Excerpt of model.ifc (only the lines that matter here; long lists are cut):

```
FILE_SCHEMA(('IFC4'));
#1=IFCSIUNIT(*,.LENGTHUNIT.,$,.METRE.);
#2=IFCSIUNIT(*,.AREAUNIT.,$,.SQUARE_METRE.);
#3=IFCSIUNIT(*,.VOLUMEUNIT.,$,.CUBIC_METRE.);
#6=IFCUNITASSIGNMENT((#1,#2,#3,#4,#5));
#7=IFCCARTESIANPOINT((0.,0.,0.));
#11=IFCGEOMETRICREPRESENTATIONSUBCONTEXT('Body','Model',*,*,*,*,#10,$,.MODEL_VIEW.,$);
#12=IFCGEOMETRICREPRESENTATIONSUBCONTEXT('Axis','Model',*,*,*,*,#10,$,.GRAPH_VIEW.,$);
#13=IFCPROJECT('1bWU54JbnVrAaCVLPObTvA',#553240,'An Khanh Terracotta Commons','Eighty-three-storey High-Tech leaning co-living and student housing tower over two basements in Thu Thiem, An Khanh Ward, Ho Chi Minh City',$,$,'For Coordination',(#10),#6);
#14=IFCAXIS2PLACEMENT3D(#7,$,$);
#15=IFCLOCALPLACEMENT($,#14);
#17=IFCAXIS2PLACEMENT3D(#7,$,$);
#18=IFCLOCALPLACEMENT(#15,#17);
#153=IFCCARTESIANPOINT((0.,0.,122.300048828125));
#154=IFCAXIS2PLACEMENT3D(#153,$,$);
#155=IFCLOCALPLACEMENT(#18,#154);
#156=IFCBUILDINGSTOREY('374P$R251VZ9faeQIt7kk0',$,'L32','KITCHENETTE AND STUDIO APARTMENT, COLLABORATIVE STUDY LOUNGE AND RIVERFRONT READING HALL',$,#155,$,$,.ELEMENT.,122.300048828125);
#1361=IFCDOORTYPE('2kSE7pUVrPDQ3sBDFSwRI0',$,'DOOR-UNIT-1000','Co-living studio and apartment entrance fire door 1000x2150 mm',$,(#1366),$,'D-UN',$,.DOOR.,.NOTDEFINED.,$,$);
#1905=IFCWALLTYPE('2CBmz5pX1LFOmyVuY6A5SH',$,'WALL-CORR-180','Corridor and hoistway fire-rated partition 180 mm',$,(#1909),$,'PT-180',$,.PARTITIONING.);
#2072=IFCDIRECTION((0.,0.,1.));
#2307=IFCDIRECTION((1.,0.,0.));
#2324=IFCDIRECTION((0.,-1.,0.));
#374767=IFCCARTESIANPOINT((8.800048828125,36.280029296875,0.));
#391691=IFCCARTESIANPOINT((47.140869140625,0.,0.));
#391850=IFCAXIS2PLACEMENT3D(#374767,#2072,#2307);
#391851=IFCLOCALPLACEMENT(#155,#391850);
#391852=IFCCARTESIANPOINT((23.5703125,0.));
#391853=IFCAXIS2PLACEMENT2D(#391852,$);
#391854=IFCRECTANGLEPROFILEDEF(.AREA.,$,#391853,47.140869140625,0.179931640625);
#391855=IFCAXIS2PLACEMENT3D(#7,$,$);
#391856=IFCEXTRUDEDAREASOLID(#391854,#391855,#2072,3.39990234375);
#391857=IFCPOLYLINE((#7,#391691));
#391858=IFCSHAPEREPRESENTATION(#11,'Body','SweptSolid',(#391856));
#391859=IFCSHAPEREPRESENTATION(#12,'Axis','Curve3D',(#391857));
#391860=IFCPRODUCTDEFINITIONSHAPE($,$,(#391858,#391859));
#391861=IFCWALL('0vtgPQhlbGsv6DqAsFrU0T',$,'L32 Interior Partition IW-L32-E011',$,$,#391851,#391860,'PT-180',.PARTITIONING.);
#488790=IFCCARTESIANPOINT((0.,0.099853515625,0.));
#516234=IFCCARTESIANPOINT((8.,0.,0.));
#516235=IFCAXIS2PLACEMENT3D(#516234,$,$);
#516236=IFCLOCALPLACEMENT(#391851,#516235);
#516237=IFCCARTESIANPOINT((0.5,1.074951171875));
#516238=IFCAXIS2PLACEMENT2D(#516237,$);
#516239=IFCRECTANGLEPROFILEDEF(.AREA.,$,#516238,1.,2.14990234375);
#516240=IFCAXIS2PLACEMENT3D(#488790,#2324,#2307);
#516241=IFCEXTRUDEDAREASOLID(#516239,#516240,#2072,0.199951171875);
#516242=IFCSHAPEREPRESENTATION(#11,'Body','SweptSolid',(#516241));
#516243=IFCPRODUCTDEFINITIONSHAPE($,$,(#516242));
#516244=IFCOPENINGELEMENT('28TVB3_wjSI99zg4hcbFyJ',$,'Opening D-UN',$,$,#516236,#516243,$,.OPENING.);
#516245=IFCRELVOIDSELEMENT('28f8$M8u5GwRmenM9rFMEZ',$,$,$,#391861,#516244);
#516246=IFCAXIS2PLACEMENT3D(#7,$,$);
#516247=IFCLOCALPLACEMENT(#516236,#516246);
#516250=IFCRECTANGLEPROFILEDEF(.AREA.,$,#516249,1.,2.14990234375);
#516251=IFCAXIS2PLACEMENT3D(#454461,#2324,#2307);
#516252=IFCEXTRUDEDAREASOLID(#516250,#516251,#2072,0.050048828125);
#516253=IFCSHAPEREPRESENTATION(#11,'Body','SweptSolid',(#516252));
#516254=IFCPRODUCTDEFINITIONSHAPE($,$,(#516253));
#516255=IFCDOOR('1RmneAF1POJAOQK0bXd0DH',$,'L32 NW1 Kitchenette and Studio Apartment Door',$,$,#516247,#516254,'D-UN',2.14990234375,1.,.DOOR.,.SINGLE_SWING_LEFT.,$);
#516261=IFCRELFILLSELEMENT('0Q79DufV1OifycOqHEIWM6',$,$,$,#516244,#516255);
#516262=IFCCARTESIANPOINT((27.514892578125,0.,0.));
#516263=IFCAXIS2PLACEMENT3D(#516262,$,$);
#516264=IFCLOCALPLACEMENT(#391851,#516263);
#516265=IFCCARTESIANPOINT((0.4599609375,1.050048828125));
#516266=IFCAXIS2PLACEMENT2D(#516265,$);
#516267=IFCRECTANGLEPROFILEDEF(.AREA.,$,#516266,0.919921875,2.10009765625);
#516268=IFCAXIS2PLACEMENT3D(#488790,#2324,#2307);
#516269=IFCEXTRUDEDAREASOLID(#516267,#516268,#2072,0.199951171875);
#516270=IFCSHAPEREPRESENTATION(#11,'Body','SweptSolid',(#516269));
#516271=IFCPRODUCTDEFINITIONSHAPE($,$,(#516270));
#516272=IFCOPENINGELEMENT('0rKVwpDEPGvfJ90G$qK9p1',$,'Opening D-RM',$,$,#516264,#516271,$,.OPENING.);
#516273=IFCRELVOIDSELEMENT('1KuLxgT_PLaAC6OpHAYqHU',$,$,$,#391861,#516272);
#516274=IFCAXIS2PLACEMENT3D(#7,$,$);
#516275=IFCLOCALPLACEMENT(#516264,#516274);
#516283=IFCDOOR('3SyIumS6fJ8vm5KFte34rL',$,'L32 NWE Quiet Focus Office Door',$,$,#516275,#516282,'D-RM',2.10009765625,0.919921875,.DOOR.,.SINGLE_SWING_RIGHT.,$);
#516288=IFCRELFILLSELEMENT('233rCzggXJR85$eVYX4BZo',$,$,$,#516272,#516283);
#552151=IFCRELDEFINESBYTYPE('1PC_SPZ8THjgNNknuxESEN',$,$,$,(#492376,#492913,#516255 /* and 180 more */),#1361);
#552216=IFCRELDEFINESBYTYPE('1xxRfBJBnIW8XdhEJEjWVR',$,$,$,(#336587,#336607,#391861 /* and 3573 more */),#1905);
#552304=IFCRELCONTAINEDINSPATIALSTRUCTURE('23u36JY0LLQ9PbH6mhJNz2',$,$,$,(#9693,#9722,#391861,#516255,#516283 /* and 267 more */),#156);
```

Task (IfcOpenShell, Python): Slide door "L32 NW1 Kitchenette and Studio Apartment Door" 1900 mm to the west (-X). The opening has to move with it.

```python
import ifcopenshell
import ifcopenshell.api.geometry
import ifcopenshell.util.placement

model = ifcopenshell.open("model.ifc")

door = model.by_guid("1RmneAF1POJAOQK0bXd0DH")
opening = door.FillsVoids[0].RelatingOpeningElement
wall = opening.VoidsElements[0].RelatingBuildingElement

wall_matrix = ifcopenshell.util.placement.get_local_placement(wall.ObjectPlacement)
shift = wall_matrix[:3, 0] * -1.9
before = ifcopenshell.util.placement.get_local_placement(door.ObjectPlacement)[:3, 3].copy()

# The door is placed relative to its opening, so it follows when the opening moves.
matrix = ifcopenshell.util.placement.get_local_placement(opening.ObjectPlacement)
matrix[:3, 3] += shift
ifcopenshell.api.geometry.edit_object_placement(
    model, product=opening, matrix=matrix, is_si=False, should_transform_children=True
)

after = ifcopenshell.util.placement.get_local_placement(door.ObjectPlacement)[:3, 3]
print("door moved by", (after - before).round(3) + 0.0)

model.write("model_rev.ifc")
```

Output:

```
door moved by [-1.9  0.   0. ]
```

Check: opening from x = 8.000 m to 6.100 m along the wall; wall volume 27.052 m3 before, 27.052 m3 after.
